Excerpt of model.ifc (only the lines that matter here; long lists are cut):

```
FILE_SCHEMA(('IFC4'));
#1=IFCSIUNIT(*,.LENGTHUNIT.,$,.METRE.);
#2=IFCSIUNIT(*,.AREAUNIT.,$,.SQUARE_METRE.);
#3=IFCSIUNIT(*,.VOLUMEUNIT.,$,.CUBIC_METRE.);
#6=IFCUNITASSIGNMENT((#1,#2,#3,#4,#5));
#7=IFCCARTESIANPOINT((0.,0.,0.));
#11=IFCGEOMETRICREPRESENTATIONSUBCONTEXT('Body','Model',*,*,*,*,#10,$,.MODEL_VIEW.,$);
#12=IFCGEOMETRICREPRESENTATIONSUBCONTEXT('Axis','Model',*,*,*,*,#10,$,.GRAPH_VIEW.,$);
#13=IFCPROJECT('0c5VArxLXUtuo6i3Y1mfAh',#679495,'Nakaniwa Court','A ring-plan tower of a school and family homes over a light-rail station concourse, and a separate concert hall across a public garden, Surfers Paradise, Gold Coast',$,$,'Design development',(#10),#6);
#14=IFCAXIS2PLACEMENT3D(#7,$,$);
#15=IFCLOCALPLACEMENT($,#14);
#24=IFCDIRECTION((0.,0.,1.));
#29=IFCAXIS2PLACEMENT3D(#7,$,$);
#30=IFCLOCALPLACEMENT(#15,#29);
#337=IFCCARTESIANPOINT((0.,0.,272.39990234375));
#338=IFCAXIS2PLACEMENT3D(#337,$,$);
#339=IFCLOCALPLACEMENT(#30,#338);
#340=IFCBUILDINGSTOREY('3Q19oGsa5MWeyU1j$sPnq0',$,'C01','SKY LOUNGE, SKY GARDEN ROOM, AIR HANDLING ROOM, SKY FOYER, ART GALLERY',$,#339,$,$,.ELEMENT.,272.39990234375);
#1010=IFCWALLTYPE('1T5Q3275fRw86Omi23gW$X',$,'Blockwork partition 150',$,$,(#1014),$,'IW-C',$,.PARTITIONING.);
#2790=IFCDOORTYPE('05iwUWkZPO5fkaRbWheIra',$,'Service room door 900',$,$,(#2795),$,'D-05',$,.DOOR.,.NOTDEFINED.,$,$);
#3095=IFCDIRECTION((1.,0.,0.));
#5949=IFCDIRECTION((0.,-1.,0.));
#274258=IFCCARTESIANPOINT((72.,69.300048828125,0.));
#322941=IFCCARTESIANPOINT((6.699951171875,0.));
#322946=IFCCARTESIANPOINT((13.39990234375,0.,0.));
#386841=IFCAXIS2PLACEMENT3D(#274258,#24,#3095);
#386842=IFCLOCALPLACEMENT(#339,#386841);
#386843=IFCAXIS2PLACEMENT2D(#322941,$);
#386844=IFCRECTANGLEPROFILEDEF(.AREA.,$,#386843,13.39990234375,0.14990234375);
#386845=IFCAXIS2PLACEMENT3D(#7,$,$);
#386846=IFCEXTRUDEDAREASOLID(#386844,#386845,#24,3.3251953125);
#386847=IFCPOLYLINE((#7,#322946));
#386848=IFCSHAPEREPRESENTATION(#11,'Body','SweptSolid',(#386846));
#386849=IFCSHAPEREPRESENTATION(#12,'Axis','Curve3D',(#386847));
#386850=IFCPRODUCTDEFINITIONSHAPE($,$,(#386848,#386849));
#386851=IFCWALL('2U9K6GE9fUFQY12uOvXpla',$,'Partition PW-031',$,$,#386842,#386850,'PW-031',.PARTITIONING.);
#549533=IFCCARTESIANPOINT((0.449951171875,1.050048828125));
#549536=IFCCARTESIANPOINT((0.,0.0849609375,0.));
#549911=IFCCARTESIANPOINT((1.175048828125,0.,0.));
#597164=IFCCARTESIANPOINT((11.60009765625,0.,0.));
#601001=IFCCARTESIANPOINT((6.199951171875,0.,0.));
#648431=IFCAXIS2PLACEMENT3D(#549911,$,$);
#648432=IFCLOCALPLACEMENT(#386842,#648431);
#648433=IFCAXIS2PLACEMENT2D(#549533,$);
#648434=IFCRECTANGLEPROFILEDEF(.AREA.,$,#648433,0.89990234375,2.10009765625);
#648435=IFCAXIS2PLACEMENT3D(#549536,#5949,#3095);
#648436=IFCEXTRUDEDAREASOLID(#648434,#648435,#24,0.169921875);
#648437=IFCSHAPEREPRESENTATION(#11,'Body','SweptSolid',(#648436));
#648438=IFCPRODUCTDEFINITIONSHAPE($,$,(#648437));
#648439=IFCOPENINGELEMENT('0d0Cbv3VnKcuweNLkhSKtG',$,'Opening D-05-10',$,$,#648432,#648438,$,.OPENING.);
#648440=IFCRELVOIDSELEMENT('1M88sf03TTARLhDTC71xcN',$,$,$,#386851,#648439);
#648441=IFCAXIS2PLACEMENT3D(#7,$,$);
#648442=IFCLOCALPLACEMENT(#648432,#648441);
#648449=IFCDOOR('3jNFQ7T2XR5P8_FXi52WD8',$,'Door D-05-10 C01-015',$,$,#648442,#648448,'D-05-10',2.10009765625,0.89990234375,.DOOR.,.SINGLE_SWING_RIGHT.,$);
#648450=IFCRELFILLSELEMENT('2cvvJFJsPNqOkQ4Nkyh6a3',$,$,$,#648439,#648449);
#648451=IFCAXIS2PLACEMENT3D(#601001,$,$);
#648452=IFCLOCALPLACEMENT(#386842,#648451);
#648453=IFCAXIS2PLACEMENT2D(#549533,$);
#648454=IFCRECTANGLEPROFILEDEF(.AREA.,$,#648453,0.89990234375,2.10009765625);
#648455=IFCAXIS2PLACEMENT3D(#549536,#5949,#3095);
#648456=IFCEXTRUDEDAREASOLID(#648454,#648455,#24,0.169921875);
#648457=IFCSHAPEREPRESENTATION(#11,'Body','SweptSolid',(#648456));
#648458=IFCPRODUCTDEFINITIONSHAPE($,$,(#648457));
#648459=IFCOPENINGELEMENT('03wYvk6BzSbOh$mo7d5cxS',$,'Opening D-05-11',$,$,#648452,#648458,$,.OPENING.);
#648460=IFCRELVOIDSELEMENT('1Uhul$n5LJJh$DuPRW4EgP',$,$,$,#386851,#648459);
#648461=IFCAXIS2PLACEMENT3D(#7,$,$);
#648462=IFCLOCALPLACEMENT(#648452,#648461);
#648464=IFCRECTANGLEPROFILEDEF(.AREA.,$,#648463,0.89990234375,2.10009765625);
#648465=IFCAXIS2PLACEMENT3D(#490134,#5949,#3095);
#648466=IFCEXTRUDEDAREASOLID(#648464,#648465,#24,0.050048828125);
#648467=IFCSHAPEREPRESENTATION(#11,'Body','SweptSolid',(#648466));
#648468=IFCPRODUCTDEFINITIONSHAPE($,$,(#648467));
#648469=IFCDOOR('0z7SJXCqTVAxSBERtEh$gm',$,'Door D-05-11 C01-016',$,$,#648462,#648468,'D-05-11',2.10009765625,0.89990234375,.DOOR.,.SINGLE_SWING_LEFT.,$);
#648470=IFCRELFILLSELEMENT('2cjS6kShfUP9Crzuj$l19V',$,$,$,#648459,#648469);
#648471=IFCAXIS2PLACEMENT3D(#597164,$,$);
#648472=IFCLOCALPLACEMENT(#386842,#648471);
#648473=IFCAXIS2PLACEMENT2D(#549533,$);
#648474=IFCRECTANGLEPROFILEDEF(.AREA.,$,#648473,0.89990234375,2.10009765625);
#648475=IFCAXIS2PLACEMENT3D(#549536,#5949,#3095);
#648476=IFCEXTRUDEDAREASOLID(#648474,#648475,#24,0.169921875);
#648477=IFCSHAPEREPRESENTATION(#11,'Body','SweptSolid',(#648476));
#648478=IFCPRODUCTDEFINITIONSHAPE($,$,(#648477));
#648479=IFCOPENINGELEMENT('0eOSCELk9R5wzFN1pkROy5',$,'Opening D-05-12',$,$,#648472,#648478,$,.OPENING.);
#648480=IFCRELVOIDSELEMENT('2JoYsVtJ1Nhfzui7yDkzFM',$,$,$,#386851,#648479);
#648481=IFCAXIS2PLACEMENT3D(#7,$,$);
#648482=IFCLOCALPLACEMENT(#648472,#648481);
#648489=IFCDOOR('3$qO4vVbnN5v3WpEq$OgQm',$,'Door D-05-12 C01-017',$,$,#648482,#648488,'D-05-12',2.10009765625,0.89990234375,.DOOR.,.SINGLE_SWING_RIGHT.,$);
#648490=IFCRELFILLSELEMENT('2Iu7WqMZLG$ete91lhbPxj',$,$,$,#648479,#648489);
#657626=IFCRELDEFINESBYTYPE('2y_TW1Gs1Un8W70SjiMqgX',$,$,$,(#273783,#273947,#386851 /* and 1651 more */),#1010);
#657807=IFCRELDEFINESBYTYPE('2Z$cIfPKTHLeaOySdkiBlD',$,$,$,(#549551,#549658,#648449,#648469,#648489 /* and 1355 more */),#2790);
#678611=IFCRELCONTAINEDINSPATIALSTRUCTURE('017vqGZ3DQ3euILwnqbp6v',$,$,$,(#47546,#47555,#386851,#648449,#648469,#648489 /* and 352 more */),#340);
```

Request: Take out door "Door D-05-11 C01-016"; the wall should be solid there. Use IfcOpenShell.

```python
import ifcopenshell
import ifcopenshell.api.feature
import ifcopenshell.api.root
import ifcopenshell.geom
import ifcopenshell.util.shape

model = ifcopenshell.open("model.ifc")
settings = ifcopenshell.geom.settings()


def volume(element):
    """Net volume in cubic metres, openings subtracted."""
    shape = ifcopenshell.geom.create_shape(settings, element)
    return ifcopenshell.util.shape.get_volume(shape.geometry)


door = model.by_guid("0z7SJXCqTVAxSBERtEh$gm")
opening = door.FillsVoids[0].RelatingOpeningElement
wall = opening.VoidsElements[0].RelatingBuildingElement
before = volume(wall)

ifcopenshell.api.root.remove_product(model, product=door)
ifcopenshell.api.feature.remove_feature(model, feature=opening)

after = volume(wall)

print(f"wall volume {before:.3f} -> {after:.3f} m3")

model.write("model-out.ifc")
```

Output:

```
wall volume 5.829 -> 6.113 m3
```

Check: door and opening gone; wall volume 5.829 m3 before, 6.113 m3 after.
